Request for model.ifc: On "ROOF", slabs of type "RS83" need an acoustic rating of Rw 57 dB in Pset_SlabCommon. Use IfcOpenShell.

First a look at what the model holds.

```python
import ifcopenshell
import ifcopenshell.util.element

model = ifcopenshell.open("model.ifc")
print(model.schema)
storey = next(s for s in model.by_type("IfcBuildingStorey") if s.Name == "ROOF")
slabs = [e for e in ifcopenshell.util.element.get_decomposition(storey) if e.is_a("IfcSlab")]
seen = {}
for e in slabs:
    element_type = ifcopenshell.util.element.get_type(e)
    key = (element_type.Name if element_type != e and element_type else None, ifcopenshell.util.element.get_pset(e, "Pset_SlabCommon", "AcousticRating"))
    seen[key] = seen.get(key, 0) + 1
for (name, value), count in sorted(seen.items(), key=str):
    print(count, "x", name, "|", value)
```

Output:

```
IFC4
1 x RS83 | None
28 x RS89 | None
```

```python
import ifcopenshell
import ifcopenshell.api.pset
import ifcopenshell.util.element

model = ifcopenshell.open("model.ifc")

storey = next(s for s in model.by_type("IfcBuildingStorey") if s.Name == "ROOF")
slabs = [e for e in ifcopenshell.util.element.get_decomposition(storey) if e.is_a("IfcSlab")]

count = 0
for e in slabs:
    element_type = ifcopenshell.util.element.get_type(e)
    if element_type in (None, e) or element_type.Name != "RS83":
        continue
    # add_pset returns the element's existing set when there is one.
    pset = ifcopenshell.api.pset.add_pset(model, product=e, name="Pset_SlabCommon")
    ifcopenshell.api.pset.edit_pset(model, pset=pset, properties={"AcousticRating": "Rw 57 dB"})
    count += 1

print(count, "slabs updated")

model.write("model_v2.ifc")
```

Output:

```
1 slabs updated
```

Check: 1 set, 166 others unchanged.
